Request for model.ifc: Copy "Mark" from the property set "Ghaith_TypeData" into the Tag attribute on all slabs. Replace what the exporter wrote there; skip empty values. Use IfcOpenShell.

First a look at what the model holds.

```python
import ifcopenshell
import ifcopenshell.util.element

model = ifcopenshell.open("model.ifc")
print(model.schema)
slabs = model.by_type("IfcSlab")
print(len(slabs), "slabs")
for e in slabs[:8]:
    source = ifcopenshell.util.element.get_pset(e, "Ghaith_TypeData", "Mark")
    target = e.Tag
    print(e.id(), repr(source), repr(target), sep=" | ")
```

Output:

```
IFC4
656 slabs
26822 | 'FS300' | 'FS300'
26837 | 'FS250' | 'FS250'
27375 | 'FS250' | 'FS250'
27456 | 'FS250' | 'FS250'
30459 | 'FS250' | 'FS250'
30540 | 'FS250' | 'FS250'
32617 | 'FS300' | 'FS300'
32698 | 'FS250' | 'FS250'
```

```python
import ifcopenshell
import ifcopenshell.util.element

model = ifcopenshell.open("model.ifc")

count = 0
for e in model.by_type("IfcSlab"):
    value = ifcopenshell.util.element.get_pset(e, "Ghaith_TypeData", "Mark")
    current = e.Tag
    if not value or not value.strip() or current == value:
        continue
    e.Tag = value
    count += 1

print(count, "slabs updated")

model.write("model_rev.ifc")
```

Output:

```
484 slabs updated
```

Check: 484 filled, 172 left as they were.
